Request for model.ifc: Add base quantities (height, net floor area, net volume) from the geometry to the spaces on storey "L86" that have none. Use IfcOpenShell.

First a look at what the model holds.

```python
import ifcopenshell
import ifcopenshell.util.element
import ifcopenshell.util.unit

model = ifcopenshell.open("model.ifc")
print(model.schema)
for unit_type in ("LENGTHUNIT", "AREAUNIT", "VOLUMEUNIT"):
    print(unit_type, ifcopenshell.util.unit.calculate_unit_scale(model, unit_type))
storey = next(s for s in model.by_type("IfcBuildingStorey") if s.Name == "L86")
spaces = [e for e in ifcopenshell.util.element.get_decomposition(storey) if e.is_a("IfcSpace")]
for e in sorted(spaces, key=lambda e: e.id()):
    print(e.id(), e.is_a(), e.Name, list(ifcopenshell.util.element.get_psets(e, qtos_only=True)), sep=" | ")
```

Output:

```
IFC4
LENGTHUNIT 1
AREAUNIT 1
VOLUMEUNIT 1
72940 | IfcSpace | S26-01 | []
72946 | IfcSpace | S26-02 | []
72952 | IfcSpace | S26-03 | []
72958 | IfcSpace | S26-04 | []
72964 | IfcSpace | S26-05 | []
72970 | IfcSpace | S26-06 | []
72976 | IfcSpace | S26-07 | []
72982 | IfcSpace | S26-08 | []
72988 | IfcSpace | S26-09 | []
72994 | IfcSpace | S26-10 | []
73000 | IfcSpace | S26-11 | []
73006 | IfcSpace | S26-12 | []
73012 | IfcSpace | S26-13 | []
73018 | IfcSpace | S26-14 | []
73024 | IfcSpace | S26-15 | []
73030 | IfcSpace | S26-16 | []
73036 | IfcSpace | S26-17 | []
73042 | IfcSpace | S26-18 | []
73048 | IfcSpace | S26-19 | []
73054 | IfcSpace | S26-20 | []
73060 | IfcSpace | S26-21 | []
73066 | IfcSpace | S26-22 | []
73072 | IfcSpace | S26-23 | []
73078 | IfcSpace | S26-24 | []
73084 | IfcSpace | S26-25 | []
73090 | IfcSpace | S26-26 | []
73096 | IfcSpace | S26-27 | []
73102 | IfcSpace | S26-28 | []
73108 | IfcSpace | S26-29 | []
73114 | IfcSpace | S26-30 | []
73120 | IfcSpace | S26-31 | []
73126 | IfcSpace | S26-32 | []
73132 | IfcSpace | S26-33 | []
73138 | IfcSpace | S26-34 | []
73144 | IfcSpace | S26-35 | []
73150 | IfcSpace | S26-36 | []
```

```python
import ifcopenshell
import ifcopenshell.api.pset
import ifcopenshell.geom
import ifcopenshell.util.element
import ifcopenshell.util.shape
import ifcopenshell.util.unit

model = ifcopenshell.open("model.ifc")
unit_scale = ifcopenshell.util.unit.calculate_unit_scale(model)
area_scale = ifcopenshell.util.unit.calculate_unit_scale(model, "AREAUNIT")
volume_scale = ifcopenshell.util.unit.calculate_unit_scale(model, "VOLUMEUNIT")
settings = ifcopenshell.geom.settings()

storey = next(s for s in model.by_type("IfcBuildingStorey") if s.Name == "L86")
spaces = [e for e in ifcopenshell.util.element.get_decomposition(storey) if e.is_a("IfcSpace")]

for e in sorted(spaces, key=lambda e: e.id()):
    if ifcopenshell.util.element.get_psets(e, qtos_only=True, should_inherit=False):
        continue
    # Geometry comes back in metres, in the element's own axes.
    shape = ifcopenshell.geom.create_shape(settings, e)
    values = {
        "Height": ifcopenshell.util.shape.get_z(shape.geometry) / unit_scale,
        "NetFloorArea": ifcopenshell.util.shape.get_footprint_area(shape.geometry) / area_scale,
        "NetVolume": ifcopenshell.util.shape.get_volume(shape.geometry) / volume_scale,
    }
    qto = ifcopenshell.api.pset.add_qto(model, product=e, name="Qto_SpaceBaseQuantities")
    ifcopenshell.api.pset.edit_qto(model, qto=qto, properties=values)
    print(e.id(), {k: round(v, 3) for k, v in values.items()})

model.write("model_v2.ifc")
```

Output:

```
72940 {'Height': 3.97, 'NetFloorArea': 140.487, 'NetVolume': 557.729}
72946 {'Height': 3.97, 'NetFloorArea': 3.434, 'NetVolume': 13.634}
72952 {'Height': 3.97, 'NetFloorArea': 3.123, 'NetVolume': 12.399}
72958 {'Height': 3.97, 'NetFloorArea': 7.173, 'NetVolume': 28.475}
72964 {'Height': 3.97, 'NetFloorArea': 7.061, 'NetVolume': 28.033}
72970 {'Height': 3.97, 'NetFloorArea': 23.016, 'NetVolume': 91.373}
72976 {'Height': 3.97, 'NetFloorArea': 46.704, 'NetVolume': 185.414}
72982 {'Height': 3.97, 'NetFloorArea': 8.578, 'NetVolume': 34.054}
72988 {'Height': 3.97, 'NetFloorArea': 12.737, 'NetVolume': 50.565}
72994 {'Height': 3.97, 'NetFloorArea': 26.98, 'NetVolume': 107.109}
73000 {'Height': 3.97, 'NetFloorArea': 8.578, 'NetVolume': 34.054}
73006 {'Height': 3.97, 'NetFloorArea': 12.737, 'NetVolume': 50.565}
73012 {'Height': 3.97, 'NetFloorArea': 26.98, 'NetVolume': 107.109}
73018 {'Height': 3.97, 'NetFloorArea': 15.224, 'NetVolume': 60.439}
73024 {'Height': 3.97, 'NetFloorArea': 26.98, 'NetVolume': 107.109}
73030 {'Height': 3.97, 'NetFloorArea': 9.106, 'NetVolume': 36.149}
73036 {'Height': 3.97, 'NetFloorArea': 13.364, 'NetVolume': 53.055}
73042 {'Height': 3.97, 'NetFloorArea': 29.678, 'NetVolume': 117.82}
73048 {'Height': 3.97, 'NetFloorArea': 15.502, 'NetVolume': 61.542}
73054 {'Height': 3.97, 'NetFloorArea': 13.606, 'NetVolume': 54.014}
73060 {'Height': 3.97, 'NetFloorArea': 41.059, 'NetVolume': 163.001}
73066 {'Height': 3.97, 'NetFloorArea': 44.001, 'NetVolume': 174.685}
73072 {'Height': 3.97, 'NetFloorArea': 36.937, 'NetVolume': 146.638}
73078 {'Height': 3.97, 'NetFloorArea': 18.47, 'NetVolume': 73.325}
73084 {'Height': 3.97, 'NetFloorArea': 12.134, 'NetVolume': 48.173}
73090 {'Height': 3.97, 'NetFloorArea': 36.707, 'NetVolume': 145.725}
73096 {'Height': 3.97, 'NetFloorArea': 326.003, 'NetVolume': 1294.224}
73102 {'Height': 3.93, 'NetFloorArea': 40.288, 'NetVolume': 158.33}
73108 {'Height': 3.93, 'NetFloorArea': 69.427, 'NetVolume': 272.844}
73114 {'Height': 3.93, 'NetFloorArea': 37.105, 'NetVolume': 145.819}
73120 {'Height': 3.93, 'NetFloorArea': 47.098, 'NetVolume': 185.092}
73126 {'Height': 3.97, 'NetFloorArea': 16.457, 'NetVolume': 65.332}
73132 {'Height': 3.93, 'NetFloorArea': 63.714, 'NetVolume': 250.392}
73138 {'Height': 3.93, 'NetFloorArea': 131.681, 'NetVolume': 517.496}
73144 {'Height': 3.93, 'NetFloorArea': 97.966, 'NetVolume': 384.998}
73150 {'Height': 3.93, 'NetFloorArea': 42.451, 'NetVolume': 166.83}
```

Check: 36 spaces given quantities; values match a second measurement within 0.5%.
